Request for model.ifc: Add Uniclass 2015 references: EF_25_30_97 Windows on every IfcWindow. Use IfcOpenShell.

First a look at what the model holds.

```python
import ifcopenshell

model = ifcopenshell.open("model.ifc")
print(model.schema)
print("classifications:", [c.Name for c in model.by_type("IfcClassification")])
for ifc_class in ("IfcDoor", "IfcRoof", "IfcStair", "IfcWall", "IfcWindow"):
    print(ifc_class, len(model.by_type(ifc_class)))
```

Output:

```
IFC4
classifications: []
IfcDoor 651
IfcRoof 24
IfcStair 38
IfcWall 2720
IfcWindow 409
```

```python
import ifcopenshell
import ifcopenshell.api.classification

model = ifcopenshell.open("model.ifc")

system = ifcopenshell.api.classification.add_classification(model, classification="Uniclass 2015")

codes = {
    "IfcWindow": ("EF_25_30_97", "Windows"),
}
for ifc_class, (code, name) in codes.items():
    products = model.by_type(ifc_class)
    ifcopenshell.api.classification.add_reference(
        model, products=products, classification=system, identification=code, name=name
    )
    print(code, len(products))

model.write("model_edited.ifc")
```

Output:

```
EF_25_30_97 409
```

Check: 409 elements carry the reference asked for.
